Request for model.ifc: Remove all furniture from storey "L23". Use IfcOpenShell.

First a look at what the model holds.

```python
import ifcopenshell
import ifcopenshell.util.element

model = ifcopenshell.open("model.ifc")
print(model.schema)
storey = next(s for s in model.by_type("IfcBuildingStorey") if s.Name == "L23")
furniture = [e for e in ifcopenshell.util.element.get_decomposition(storey) if e.is_a("IfcFurnishingElement")]
seen = {}
for e in furniture:
    element_type = ifcopenshell.util.element.get_type(e)
    name = element_type.Name if element_type not in (None, e) else None
    seen[name] = seen.get(name, 0) + 1
for name, count in sorted(seen.items(), key=str):
    print(count, "x", name)
```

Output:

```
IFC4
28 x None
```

```python
import ifcopenshell
import ifcopenshell.api.root
import ifcopenshell.util.element

model = ifcopenshell.open("model.ifc")

storey = next(s for s in model.by_type("IfcBuildingStorey") if s.Name == "L23")
furniture = [e for e in ifcopenshell.util.element.get_decomposition(storey) if e.is_a("IfcFurnishingElement")]

for e in furniture:
    ifcopenshell.api.root.remove_product(model, product=e)
print(len(furniture), "removed")

model.write("model-out.ifc")
```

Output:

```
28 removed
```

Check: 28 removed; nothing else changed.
